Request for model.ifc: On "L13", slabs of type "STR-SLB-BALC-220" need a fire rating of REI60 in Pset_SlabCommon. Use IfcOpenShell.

First a look at what the model holds.

```python
import ifcopenshell
import ifcopenshell.util.element

model = ifcopenshell.open("model.ifc")
print(model.schema)
storey = next(s for s in model.by_type("IfcBuildingStorey") if s.Name == "L13")
slabs = [e for e in ifcopenshell.util.element.get_decomposition(storey) if e.is_a("IfcSlab")]
seen = {}
for e in slabs:
    element_type = ifcopenshell.util.element.get_type(e)
    key = (element_type.Name if element_type != e and element_type else None, ifcopenshell.util.element.get_pset(e, "Pset_SlabCommon", "FireRating"))
    seen[key] = seen.get(key, 0) + 1
for (name, value), count in sorted(seen.items(), key=str):
    print(count, "x", name, "|", value)
```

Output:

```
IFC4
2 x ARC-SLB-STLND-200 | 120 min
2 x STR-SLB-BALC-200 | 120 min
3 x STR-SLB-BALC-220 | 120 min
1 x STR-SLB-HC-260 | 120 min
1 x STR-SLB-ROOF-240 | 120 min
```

```python
import ifcopenshell
import ifcopenshell.api.pset
import ifcopenshell.util.element

model = ifcopenshell.open("model.ifc")

storey = next(s for s in model.by_type("IfcBuildingStorey") if s.Name == "L13")
slabs = [e for e in ifcopenshell.util.element.get_decomposition(storey) if e.is_a("IfcSlab")]

count = 0
for e in slabs:
    element_type = ifcopenshell.util.element.get_type(e)
    if element_type in (None, e) or element_type.Name != "STR-SLB-BALC-220":
        continue
    # add_pset returns the element's existing set when there is one.
    pset = ifcopenshell.api.pset.add_pset(model, product=e, name="Pset_SlabCommon")
    ifcopenshell.api.pset.edit_pset(model, pset=pset, properties={"FireRating": "REI60"})
    count += 1

print(count, "slabs updated")

model.write("model_rev.ifc")
```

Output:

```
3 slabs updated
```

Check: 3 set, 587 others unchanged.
